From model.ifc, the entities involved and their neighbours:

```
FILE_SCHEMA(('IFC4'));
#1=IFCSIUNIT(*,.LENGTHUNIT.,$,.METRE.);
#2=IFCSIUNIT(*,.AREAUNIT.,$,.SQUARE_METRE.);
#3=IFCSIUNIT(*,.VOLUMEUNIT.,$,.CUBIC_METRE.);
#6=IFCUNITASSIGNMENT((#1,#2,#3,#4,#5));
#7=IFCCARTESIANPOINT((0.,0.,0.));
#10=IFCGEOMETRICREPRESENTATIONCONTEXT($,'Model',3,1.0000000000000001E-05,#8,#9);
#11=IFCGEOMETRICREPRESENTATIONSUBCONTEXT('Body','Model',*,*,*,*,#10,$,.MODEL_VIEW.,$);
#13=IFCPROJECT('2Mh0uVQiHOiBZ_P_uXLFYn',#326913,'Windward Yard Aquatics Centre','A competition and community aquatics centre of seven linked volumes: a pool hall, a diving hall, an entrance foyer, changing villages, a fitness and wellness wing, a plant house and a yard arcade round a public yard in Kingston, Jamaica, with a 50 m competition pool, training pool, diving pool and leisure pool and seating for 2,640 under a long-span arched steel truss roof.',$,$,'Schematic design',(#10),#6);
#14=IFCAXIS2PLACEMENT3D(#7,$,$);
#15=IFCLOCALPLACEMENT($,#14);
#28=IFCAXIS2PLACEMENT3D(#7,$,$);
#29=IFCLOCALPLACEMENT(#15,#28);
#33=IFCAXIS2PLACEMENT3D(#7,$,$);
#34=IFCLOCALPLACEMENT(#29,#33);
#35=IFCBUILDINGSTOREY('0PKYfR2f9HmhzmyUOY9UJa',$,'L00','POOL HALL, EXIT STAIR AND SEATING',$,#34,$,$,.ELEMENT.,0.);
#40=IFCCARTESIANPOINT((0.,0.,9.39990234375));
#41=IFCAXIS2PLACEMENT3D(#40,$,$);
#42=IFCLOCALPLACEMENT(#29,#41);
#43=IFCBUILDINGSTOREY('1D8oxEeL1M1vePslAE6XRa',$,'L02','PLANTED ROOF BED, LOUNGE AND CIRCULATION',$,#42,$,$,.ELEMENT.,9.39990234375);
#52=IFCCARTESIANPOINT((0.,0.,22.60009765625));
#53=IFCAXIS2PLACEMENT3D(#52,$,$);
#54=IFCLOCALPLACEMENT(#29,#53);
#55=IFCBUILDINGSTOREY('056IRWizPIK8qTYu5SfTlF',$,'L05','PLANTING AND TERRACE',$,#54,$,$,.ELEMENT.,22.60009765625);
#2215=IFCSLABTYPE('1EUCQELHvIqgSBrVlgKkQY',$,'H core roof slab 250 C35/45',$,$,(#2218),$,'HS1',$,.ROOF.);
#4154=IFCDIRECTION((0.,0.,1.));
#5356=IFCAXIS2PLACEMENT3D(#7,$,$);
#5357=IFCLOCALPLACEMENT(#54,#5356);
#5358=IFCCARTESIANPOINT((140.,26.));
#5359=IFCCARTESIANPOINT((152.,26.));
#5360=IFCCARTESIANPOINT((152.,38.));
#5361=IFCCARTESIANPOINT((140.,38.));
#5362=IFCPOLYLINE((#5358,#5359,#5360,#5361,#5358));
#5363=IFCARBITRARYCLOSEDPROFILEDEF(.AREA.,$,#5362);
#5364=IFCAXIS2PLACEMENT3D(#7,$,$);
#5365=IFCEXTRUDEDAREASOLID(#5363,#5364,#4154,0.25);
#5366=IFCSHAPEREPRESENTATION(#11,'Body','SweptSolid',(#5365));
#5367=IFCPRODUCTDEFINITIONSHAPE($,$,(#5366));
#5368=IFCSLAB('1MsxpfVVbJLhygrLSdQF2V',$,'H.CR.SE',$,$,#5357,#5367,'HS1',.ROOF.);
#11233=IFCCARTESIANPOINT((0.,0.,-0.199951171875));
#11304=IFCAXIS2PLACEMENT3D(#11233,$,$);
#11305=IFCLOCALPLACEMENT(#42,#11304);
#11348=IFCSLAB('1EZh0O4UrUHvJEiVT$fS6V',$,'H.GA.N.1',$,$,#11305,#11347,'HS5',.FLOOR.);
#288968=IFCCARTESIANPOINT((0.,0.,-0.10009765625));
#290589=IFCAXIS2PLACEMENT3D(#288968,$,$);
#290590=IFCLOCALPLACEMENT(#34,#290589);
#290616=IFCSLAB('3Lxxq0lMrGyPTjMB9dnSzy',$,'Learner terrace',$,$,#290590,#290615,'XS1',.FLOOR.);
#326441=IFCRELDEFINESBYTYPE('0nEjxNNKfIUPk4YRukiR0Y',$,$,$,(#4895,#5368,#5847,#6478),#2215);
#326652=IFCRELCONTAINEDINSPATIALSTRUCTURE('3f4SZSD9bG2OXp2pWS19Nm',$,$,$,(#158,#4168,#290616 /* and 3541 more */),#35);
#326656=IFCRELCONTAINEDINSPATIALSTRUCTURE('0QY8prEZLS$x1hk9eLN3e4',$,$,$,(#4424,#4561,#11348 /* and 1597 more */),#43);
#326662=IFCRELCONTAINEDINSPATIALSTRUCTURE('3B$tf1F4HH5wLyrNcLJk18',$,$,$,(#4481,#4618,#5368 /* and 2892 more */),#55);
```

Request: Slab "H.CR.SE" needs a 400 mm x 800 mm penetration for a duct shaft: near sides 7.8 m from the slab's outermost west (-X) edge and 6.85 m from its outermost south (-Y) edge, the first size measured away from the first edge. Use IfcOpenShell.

```python
import numpy as np
import ifcopenshell
import ifcopenshell.api.feature
import ifcopenshell.api.geometry
import ifcopenshell.api.root
import ifcopenshell.geom
import ifcopenshell.util.placement
import ifcopenshell.util.representation
import ifcopenshell.util.shape
import ifcopenshell.util.unit

model = ifcopenshell.open("model.ifc")
unit_scale = ifcopenshell.util.unit.calculate_unit_scale(model)
settings = ifcopenshell.geom.settings()


def volume(element):
    """Net volume in cubic metres, openings subtracted."""
    shape = ifcopenshell.geom.create_shape(settings, element)
    return ifcopenshell.util.shape.get_volume(shape.geometry)


slab = model.by_id(5368)
before = volume(slab)

# Extent in the slab's own axes, in metres. The edges named are its -X and -Y sides.
slab_shape = ifcopenshell.geom.create_shape(settings, slab)
vertices = ifcopenshell.util.shape.get_vertices(slab_shape.geometry)
x_min, y_min, bottom = vertices.min(axis=0)
top = vertices[:, 2].max()

opening = ifcopenshell.api.root.create_entity(model, ifc_class="IfcOpeningElement", name="Duct shaft opening", predefined_type="OPENING")
context = ifcopenshell.util.representation.get_context(model, "Model", "Body", "MODEL_VIEW")
width, depth = 0.4, 0.8
outline = [(0.0, 0.0), (width, 0.0), (width, depth), (0.0, depth), (0.0, 0.0)]
# Overshoot both faces by 50 mm so the cut is clean.
shape = ifcopenshell.api.geometry.add_slab_representation(
    model, context=context, depth=top - bottom + 0.1, polyline=outline
)
ifcopenshell.api.geometry.assign_representation(model, product=opening, representation=shape)

matrix = ifcopenshell.util.placement.get_local_placement(slab.ObjectPlacement)
matrix[:, 3] = matrix @ np.append(np.array([x_min + 7.8, y_min + 6.85, bottom - 0.05]) / unit_scale, 1.0)
ifcopenshell.api.geometry.edit_object_placement(model, product=opening, matrix=matrix, is_si=False)
ifcopenshell.api.feature.add_feature(model, feature=opening, element=slab)

after = volume(slab)

print(f"slab volume {before:.3f} -> {after:.3f} m3")

model.write("model-out.ifc")
```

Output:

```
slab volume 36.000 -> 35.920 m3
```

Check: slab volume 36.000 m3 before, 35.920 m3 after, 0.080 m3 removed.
